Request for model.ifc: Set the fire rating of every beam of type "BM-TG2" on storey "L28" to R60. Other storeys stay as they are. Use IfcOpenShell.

First a look at what the model holds.

```python
import ifcopenshell
import ifcopenshell.util.element

model = ifcopenshell.open("model.ifc")
print(model.schema)
storey = next(s for s in model.by_type("IfcBuildingStorey") if s.Name == "L28")
beams = [e for e in ifcopenshell.util.element.get_decomposition(storey) if e.is_a("IfcBeam")]
seen = {}
for e in beams:
    element_type = ifcopenshell.util.element.get_type(e)
    key = (element_type.Name if element_type != e and element_type else None, ifcopenshell.util.element.get_pset(e, "Pset_BeamCommon", "FireRating"))
    seen[key] = seen.get(key, 0) + 1
for (name, value), count in sorted(seen.items(), key=str):
    print(count, "x", name, "|", value)
```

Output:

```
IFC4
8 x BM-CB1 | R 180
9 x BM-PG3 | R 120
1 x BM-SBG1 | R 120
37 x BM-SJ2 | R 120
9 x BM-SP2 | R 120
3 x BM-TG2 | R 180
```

```python
import ifcopenshell
import ifcopenshell.api.pset
import ifcopenshell.util.element

model = ifcopenshell.open("model.ifc")

storey = next(s for s in model.by_type("IfcBuildingStorey") if s.Name == "L28")
beams = [e for e in ifcopenshell.util.element.get_decomposition(storey) if e.is_a("IfcBeam")]

count = 0
for e in beams:
    element_type = ifcopenshell.util.element.get_type(e)
    if element_type in (None, e) or element_type.Name != "BM-TG2":
        continue
    # add_pset returns the element's existing set when there is one.
    pset = ifcopenshell.api.pset.add_pset(model, product=e, name="Pset_BeamCommon")
    ifcopenshell.api.pset.edit_pset(model, pset=pset, properties={"FireRating": "R60"})
    count += 1

print(count, "beams updated")

model.write("model_rev.ifc")
```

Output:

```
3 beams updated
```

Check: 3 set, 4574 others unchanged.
